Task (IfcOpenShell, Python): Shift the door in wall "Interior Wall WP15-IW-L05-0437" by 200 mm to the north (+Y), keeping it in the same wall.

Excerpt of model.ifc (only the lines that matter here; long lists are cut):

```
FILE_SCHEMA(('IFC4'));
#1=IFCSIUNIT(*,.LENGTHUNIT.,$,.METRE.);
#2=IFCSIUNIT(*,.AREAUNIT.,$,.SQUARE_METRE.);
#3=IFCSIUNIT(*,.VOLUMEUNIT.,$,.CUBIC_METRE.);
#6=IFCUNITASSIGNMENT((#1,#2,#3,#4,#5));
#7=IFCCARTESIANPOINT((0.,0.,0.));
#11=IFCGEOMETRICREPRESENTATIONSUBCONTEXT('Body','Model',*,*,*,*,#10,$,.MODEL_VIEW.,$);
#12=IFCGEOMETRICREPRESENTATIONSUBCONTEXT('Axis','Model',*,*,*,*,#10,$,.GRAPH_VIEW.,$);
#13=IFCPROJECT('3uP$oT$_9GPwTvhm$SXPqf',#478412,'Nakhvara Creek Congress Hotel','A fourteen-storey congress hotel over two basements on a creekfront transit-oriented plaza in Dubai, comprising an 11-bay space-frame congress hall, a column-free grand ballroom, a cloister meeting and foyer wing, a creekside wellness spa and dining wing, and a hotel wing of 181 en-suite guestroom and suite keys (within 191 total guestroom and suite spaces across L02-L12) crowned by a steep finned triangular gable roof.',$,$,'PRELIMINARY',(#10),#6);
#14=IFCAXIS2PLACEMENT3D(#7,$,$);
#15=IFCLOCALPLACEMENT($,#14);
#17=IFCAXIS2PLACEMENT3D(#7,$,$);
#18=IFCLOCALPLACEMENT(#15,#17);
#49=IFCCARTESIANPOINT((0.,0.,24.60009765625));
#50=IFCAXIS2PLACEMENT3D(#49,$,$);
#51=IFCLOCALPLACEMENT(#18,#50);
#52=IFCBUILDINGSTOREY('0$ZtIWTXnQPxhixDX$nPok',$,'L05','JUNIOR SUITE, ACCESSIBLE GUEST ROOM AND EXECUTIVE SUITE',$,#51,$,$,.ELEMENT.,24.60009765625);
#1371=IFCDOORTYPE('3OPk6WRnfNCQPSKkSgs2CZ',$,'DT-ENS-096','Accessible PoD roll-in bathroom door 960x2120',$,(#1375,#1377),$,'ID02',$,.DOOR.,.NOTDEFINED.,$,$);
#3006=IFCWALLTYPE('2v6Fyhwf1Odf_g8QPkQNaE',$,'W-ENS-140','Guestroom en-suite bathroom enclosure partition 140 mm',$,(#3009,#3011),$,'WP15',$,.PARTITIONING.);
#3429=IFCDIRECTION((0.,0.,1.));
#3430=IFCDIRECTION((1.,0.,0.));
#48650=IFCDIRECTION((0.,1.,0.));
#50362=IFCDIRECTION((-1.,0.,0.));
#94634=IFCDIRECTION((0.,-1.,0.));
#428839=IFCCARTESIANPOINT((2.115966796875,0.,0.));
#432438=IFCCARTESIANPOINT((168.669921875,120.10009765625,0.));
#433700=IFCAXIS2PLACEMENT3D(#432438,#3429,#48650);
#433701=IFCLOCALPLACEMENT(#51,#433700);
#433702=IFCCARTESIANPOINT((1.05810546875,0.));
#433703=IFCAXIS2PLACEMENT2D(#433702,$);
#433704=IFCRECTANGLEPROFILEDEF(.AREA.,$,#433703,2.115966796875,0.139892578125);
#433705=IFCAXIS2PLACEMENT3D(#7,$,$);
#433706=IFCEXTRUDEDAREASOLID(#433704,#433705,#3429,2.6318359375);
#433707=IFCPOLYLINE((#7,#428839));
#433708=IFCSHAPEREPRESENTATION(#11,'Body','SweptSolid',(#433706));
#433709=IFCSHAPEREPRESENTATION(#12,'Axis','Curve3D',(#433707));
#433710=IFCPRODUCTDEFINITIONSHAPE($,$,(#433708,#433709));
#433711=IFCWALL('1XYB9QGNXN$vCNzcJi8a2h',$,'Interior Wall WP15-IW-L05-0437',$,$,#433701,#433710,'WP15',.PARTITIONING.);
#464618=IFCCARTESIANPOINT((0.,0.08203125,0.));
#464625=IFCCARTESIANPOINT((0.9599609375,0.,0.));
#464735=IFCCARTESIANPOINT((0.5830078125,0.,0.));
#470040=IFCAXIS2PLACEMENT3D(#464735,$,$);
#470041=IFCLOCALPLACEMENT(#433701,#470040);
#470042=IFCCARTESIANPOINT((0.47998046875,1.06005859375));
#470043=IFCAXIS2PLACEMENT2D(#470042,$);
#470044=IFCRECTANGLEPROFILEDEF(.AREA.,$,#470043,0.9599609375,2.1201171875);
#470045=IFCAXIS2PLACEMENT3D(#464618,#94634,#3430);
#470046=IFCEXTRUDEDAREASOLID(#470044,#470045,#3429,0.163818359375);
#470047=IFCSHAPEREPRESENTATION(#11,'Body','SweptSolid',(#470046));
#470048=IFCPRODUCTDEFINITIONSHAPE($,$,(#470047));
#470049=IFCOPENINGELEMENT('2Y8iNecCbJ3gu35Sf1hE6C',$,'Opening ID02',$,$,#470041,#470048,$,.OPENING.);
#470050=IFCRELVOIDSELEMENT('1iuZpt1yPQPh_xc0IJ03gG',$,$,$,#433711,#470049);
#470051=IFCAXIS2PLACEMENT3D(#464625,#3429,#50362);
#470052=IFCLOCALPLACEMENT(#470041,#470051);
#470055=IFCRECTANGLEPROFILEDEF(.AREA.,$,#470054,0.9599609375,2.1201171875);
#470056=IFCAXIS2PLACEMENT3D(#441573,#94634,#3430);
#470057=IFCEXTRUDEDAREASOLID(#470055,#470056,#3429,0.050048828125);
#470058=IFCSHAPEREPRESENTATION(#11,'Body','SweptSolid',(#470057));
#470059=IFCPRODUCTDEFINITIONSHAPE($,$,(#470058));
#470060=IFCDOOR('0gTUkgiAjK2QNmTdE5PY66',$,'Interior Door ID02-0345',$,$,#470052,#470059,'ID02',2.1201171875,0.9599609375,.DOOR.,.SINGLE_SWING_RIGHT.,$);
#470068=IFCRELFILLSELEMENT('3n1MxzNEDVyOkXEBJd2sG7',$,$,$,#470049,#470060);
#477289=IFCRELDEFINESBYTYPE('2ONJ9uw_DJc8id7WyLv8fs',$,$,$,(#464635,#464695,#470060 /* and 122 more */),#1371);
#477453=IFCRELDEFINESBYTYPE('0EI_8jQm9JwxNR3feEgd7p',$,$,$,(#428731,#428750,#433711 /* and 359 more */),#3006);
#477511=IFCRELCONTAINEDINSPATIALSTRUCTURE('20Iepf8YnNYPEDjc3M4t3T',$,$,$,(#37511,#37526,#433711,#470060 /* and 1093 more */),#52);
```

```python
import ifcopenshell
import ifcopenshell.api.geometry
import ifcopenshell.util.placement

model = ifcopenshell.open("model.ifc")

door = model.by_id(470060)
opening = door.FillsVoids[0].RelatingOpeningElement
wall = opening.VoidsElements[0].RelatingBuildingElement

wall_matrix = ifcopenshell.util.placement.get_local_placement(wall.ObjectPlacement)
shift = wall_matrix[:3, 0] * 0.2
before = ifcopenshell.util.placement.get_local_placement(door.ObjectPlacement)[:3, 3].copy()

# The door is placed relative to its opening, so it follows when the opening moves.
matrix = ifcopenshell.util.placement.get_local_placement(opening.ObjectPlacement)
matrix[:3, 3] += shift
ifcopenshell.api.geometry.edit_object_placement(
    model, product=opening, matrix=matrix, is_si=False, should_transform_children=True
)

after = ifcopenshell.util.placement.get_local_placement(door.ObjectPlacement)[:3, 3]
print("door moved by", (after - before).round(3) + 0.0)

model.write("model_rev.ifc")
```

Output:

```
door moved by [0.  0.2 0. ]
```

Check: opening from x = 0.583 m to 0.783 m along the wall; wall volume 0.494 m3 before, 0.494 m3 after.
